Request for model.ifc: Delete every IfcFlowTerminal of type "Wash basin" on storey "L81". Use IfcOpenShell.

First a look at what the model holds.

```python
import ifcopenshell
import ifcopenshell.util.element

model = ifcopenshell.open("model.ifc")
print(model.schema)
storey = next(s for s in model.by_type("IfcBuildingStorey") if s.Name == "L81")
terminals = [e for e in ifcopenshell.util.element.get_decomposition(storey) if e.is_a("IfcFlowTerminal")]
seen = {}
for e in terminals:
    element_type = ifcopenshell.util.element.get_type(e)
    name = element_type.Name if element_type not in (None, e) else None
    seen[name] = seen.get(name, 0) + 1
for name, count in sorted(seen.items(), key=str):
    print(count, "x", name)
```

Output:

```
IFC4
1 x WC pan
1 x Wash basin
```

```python
import ifcopenshell
import ifcopenshell.api.root
import ifcopenshell.util.element

model = ifcopenshell.open("model.ifc")

storey = next(s for s in model.by_type("IfcBuildingStorey") if s.Name == "L81")
terminals = [e for e in ifcopenshell.util.element.get_decomposition(storey) if e.is_a("IfcFlowTerminal")]
targets = [e for e in terminals if (t := ifcopenshell.util.element.get_type(e)) not in (None, e) and t.Name == "Wash basin"]

for e in targets:
    ifcopenshell.api.root.remove_product(model, product=e)
print(len(targets), "removed")

model.write("model-out.ifc")
```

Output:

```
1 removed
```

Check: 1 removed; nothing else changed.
